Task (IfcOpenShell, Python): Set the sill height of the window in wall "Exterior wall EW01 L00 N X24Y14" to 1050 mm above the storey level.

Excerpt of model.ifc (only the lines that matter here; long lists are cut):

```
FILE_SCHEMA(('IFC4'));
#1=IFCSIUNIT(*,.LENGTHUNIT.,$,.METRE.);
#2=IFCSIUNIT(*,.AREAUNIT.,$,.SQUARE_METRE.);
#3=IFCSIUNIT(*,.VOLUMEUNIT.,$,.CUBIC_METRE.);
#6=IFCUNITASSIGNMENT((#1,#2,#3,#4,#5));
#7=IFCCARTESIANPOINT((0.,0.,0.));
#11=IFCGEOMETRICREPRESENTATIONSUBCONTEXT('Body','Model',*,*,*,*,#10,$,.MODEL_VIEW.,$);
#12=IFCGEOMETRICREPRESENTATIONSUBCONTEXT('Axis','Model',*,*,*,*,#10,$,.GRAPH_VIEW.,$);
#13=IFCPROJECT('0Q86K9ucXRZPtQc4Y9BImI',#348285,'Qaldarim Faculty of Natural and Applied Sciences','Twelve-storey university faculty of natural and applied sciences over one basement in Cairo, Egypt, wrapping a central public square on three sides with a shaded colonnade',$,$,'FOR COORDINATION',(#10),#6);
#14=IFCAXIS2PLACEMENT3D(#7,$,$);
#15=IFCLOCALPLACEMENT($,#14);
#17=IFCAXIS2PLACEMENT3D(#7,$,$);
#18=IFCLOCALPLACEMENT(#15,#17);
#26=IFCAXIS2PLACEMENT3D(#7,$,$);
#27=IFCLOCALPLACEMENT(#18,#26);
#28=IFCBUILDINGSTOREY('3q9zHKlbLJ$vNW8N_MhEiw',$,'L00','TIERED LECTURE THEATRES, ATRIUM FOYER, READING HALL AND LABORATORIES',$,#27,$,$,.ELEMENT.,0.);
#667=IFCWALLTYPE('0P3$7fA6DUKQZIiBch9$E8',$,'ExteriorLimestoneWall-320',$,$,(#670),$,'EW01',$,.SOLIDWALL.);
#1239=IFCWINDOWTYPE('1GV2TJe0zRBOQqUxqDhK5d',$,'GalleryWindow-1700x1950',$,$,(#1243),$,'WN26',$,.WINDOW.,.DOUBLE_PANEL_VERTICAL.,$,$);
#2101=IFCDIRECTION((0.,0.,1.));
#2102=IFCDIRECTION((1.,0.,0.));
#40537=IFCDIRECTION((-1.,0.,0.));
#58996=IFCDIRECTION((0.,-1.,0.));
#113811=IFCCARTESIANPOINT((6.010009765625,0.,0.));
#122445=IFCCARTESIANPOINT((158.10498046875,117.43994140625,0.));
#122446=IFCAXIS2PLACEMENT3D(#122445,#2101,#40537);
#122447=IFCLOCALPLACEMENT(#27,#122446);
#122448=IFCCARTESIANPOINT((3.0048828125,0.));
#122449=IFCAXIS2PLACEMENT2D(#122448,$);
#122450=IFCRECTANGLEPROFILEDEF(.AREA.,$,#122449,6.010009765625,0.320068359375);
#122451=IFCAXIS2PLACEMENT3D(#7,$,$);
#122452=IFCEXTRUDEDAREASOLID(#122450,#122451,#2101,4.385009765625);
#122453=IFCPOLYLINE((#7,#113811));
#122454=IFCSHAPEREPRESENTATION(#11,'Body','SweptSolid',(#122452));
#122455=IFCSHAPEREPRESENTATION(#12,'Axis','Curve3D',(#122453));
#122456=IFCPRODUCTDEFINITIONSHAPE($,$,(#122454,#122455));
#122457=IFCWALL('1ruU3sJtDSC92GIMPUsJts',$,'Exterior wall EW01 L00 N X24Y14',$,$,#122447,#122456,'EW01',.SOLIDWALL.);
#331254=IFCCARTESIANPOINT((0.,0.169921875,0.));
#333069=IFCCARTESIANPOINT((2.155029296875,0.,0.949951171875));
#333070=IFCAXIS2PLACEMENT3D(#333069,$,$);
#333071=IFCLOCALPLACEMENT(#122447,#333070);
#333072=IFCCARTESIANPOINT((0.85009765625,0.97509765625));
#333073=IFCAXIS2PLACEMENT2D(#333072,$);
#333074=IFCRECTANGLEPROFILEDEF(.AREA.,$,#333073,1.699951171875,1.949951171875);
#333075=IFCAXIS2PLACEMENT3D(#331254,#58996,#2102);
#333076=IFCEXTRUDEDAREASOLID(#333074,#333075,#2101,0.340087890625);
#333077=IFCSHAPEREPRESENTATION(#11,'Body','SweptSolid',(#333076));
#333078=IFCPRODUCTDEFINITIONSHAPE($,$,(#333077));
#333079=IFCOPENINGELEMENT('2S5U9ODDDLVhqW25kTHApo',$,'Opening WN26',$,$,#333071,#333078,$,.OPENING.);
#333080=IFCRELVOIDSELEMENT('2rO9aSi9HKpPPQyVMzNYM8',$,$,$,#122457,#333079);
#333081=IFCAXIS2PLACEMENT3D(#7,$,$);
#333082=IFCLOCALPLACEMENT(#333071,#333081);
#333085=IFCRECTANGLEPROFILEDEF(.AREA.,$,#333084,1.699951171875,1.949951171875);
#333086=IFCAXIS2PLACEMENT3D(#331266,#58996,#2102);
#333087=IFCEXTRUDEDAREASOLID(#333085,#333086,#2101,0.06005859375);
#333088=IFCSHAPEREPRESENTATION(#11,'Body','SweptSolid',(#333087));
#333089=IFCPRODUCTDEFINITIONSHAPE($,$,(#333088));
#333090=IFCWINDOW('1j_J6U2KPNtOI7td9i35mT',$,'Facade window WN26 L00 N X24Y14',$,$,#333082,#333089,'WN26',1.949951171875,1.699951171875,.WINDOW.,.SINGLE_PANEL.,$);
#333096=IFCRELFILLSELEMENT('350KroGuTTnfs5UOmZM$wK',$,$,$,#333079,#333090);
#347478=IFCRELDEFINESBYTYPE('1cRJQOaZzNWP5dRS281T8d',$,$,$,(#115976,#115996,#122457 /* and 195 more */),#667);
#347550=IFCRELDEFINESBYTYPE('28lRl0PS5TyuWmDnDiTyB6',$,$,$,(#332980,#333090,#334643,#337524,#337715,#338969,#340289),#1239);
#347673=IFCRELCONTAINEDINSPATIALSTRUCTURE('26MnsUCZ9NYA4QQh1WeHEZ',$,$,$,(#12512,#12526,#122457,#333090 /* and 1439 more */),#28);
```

```python
import numpy as np
import ifcopenshell
import ifcopenshell.api.geometry
import ifcopenshell.geom
import ifcopenshell.util.element
import ifcopenshell.util.placement
import ifcopenshell.util.shape
import ifcopenshell.util.unit

model = ifcopenshell.open("model.ifc")
unit_scale = ifcopenshell.util.unit.calculate_unit_scale(model)

window = model.by_guid("1j_J6U2KPNtOI7td9i35mT")
opening = window.FillsVoids[0].RelatingOpeningElement
storey = ifcopenshell.util.element.get_container(window, ifc_class="IfcBuildingStorey")
level = ifcopenshell.util.placement.get_local_placement(storey.ObjectPlacement)[2, 3]

# The opening's origin need not be at the sill, so measure its lowest point.
shape = ifcopenshell.geom.create_shape(ifcopenshell.geom.settings(), opening)
bottom = ifcopenshell.util.shape.get_shape_bottom_elevation(shape, shape.geometry) / unit_scale
dz = level + 1.05 - bottom

shift = np.array([0.0, 0.0, dz])
# The window is placed relative to its opening, so it follows when the opening moves.
matrix = ifcopenshell.util.placement.get_local_placement(opening.ObjectPlacement)
matrix[:3, 3] += shift
ifcopenshell.api.geometry.edit_object_placement(
    model, product=opening, matrix=matrix, is_si=False, should_transform_children=True
)

print(f"moved by {dz * unit_scale:+.3f} m")

model.write("model-out.ifc")
```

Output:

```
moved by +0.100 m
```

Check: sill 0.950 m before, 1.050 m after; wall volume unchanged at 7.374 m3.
